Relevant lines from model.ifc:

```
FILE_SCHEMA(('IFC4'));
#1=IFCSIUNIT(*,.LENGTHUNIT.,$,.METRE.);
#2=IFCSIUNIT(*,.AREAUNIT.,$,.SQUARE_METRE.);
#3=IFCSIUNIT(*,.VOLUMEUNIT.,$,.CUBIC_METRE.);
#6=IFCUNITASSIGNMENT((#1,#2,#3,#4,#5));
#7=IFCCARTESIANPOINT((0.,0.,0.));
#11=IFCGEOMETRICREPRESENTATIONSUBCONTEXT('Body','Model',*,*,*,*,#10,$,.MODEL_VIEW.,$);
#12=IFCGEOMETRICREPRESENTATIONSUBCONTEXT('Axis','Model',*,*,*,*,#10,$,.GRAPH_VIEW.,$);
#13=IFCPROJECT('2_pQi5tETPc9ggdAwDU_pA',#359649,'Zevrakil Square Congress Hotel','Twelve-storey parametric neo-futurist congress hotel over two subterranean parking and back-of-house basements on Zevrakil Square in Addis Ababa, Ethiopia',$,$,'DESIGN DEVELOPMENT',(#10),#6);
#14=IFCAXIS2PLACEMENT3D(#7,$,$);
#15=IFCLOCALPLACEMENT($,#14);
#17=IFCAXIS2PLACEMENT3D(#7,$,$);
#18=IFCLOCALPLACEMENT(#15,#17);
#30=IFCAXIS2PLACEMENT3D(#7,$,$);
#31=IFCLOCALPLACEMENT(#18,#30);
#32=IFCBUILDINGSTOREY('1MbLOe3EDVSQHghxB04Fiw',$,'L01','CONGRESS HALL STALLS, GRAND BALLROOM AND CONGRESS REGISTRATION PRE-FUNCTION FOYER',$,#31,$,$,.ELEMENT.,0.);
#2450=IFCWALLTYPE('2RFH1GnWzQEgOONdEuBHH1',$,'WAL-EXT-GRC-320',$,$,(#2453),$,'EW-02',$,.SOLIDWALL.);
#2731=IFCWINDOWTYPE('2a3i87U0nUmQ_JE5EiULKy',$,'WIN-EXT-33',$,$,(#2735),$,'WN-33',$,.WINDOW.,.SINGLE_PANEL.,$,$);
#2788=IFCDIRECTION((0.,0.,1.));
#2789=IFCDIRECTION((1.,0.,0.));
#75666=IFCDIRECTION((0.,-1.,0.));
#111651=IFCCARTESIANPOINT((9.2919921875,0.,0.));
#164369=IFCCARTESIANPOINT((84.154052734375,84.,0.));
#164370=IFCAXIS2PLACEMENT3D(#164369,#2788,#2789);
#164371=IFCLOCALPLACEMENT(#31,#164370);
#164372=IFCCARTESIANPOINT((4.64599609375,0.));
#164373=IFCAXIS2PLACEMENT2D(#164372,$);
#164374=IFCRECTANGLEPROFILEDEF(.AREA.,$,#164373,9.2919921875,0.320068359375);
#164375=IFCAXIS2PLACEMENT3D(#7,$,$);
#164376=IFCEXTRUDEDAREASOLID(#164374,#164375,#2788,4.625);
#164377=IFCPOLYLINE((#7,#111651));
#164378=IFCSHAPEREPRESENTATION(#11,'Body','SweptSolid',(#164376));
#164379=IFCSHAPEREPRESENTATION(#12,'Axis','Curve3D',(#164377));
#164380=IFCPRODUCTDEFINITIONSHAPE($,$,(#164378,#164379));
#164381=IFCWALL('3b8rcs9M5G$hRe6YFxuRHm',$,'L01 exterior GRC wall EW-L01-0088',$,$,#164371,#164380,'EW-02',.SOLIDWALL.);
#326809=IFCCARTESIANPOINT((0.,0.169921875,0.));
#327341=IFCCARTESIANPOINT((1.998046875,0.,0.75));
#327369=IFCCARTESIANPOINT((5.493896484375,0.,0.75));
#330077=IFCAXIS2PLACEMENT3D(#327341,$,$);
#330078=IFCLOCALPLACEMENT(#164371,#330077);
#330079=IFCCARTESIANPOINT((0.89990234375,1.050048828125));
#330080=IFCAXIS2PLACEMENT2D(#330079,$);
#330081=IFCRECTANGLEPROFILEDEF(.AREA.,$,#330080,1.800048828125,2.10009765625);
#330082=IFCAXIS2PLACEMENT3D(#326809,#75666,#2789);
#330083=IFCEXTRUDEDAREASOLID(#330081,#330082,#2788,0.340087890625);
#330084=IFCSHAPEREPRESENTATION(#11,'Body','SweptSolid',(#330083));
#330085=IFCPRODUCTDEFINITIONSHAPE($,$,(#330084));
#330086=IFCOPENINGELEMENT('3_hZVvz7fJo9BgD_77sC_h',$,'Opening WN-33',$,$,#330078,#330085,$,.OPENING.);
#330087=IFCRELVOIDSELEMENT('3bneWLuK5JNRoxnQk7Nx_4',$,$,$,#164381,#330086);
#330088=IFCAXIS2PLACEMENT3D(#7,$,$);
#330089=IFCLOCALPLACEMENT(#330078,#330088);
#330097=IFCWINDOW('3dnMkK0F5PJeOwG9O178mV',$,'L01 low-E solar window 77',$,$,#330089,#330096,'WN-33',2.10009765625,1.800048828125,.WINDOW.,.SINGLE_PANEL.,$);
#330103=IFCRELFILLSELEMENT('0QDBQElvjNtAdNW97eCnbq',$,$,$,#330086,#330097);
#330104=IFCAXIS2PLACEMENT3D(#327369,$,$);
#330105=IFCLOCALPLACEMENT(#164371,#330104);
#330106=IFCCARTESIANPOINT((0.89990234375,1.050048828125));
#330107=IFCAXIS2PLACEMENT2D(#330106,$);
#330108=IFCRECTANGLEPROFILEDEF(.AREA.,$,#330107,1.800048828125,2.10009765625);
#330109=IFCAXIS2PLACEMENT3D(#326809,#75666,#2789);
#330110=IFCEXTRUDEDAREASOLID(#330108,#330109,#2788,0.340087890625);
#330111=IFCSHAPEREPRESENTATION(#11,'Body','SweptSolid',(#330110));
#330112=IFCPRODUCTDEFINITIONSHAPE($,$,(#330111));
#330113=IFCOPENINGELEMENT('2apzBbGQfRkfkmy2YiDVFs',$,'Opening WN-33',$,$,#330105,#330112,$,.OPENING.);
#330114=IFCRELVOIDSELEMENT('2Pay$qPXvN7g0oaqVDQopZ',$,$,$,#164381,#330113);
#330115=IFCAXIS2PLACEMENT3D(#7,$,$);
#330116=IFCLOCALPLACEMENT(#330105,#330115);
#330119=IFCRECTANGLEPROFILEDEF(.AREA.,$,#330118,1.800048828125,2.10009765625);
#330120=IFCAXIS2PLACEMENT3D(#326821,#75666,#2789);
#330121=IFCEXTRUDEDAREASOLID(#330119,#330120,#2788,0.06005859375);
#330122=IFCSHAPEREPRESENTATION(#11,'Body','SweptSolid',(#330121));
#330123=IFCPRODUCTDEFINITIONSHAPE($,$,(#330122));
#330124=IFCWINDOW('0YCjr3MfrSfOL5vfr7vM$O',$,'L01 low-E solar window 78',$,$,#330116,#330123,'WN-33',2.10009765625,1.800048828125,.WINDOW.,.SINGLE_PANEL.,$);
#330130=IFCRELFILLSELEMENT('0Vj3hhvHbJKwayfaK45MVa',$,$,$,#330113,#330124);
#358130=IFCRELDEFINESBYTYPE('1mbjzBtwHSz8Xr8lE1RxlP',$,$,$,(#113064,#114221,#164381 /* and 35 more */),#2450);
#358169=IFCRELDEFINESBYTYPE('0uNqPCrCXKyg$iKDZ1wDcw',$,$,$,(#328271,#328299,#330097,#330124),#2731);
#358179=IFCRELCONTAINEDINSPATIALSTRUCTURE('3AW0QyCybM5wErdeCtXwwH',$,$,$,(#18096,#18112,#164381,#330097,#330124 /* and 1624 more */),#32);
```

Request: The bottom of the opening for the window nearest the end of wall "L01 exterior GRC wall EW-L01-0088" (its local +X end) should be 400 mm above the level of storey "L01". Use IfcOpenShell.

```python
import numpy as np
import ifcopenshell
import ifcopenshell.api.geometry
import ifcopenshell.geom
import ifcopenshell.util.element
import ifcopenshell.util.placement
import ifcopenshell.util.shape
import ifcopenshell.util.unit

model = ifcopenshell.open("model.ifc")
unit_scale = ifcopenshell.util.unit.calculate_unit_scale(model)

window = model.by_id(330124)
opening = window.FillsVoids[0].RelatingOpeningElement
storey = ifcopenshell.util.element.get_container(window, ifc_class="IfcBuildingStorey")
level = ifcopenshell.util.placement.get_local_placement(storey.ObjectPlacement)[2, 3]

# The opening's origin need not be at the sill, so measure its lowest point.
shape = ifcopenshell.geom.create_shape(ifcopenshell.geom.settings(), opening)
bottom = ifcopenshell.util.shape.get_shape_bottom_elevation(shape, shape.geometry) / unit_scale
dz = level + 0.4 - bottom

shift = np.array([0.0, 0.0, dz])
# The window is placed relative to its opening, so it follows when the opening moves.
matrix = ifcopenshell.util.placement.get_local_placement(opening.ObjectPlacement)
matrix[:3, 3] += shift
ifcopenshell.api.geometry.edit_object_placement(
    model, product=opening, matrix=matrix, is_si=False, should_transform_children=True
)

print(f"moved by {dz * unit_scale:+.3f} m")

model.write("model_v2.ifc")
```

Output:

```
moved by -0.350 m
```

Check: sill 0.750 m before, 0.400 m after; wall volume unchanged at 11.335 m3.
